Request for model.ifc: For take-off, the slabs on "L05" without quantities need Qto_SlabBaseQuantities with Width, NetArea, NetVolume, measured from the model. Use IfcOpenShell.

First a look at what the model holds.

```python
import ifcopenshell
import ifcopenshell.util.element
import ifcopenshell.util.unit

model = ifcopenshell.open("model.ifc")
print(model.schema)
for unit_type in ("LENGTHUNIT", "AREAUNIT", "VOLUMEUNIT"):
    print(unit_type, ifcopenshell.util.unit.calculate_unit_scale(model, unit_type))
storey = next(s for s in model.by_type("IfcBuildingStorey") if s.Name == "L05")
slabs = [e for e in ifcopenshell.util.element.get_decomposition(storey) if e.is_a("IfcSlab")]
for e in sorted(slabs, key=lambda e: e.id()):
    print(e.id(), e.is_a(), e.Name, list(ifcopenshell.util.element.get_psets(e, qtos_only=True)), sep=" | ")
```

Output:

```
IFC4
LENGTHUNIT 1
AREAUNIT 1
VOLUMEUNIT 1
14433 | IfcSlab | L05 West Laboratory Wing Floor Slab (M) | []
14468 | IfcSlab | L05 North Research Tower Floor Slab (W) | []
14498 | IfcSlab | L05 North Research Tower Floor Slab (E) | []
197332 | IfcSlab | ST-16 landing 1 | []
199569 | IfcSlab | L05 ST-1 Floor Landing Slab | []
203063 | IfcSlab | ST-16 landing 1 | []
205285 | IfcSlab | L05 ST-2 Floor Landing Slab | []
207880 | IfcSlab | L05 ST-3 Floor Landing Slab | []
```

```python
import ifcopenshell
import ifcopenshell.api.pset
import ifcopenshell.geom
import ifcopenshell.util.element
import ifcopenshell.util.shape
import ifcopenshell.util.unit

model = ifcopenshell.open("model.ifc")
unit_scale = ifcopenshell.util.unit.calculate_unit_scale(model)
area_scale = ifcopenshell.util.unit.calculate_unit_scale(model, "AREAUNIT")
volume_scale = ifcopenshell.util.unit.calculate_unit_scale(model, "VOLUMEUNIT")
settings = ifcopenshell.geom.settings()

storey = next(s for s in model.by_type("IfcBuildingStorey") if s.Name == "L05")
slabs = [e for e in ifcopenshell.util.element.get_decomposition(storey) if e.is_a("IfcSlab")]

for e in sorted(slabs, key=lambda e: e.id()):
    if ifcopenshell.util.element.get_psets(e, qtos_only=True, should_inherit=False):
        continue
    # Geometry comes back in metres, in the element's own axes.
    shape = ifcopenshell.geom.create_shape(settings, e)
    values = {
        "Width": ifcopenshell.util.shape.get_z(shape.geometry) / unit_scale,
        "NetArea": ifcopenshell.util.shape.get_footprint_area(shape.geometry) / area_scale,
        "NetVolume": ifcopenshell.util.shape.get_volume(shape.geometry) / volume_scale,
    }
    qto = ifcopenshell.api.pset.add_qto(model, product=e, name="Qto_SlabBaseQuantities")
    ifcopenshell.api.pset.edit_qto(model, qto=qto, properties=values)
    print(e.id(), {k: round(v, 3) for k, v in values.items()})

model.write("model_edited.ifc")
```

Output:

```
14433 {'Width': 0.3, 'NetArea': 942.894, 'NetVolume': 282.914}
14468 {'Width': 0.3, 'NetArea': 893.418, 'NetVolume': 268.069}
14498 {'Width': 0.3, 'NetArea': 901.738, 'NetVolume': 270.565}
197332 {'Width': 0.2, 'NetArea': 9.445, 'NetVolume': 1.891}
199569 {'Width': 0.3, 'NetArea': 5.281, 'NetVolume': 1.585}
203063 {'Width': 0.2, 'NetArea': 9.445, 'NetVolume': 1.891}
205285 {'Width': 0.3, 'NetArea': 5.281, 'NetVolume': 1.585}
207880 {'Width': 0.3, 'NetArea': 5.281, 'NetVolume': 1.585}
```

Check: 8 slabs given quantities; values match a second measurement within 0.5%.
